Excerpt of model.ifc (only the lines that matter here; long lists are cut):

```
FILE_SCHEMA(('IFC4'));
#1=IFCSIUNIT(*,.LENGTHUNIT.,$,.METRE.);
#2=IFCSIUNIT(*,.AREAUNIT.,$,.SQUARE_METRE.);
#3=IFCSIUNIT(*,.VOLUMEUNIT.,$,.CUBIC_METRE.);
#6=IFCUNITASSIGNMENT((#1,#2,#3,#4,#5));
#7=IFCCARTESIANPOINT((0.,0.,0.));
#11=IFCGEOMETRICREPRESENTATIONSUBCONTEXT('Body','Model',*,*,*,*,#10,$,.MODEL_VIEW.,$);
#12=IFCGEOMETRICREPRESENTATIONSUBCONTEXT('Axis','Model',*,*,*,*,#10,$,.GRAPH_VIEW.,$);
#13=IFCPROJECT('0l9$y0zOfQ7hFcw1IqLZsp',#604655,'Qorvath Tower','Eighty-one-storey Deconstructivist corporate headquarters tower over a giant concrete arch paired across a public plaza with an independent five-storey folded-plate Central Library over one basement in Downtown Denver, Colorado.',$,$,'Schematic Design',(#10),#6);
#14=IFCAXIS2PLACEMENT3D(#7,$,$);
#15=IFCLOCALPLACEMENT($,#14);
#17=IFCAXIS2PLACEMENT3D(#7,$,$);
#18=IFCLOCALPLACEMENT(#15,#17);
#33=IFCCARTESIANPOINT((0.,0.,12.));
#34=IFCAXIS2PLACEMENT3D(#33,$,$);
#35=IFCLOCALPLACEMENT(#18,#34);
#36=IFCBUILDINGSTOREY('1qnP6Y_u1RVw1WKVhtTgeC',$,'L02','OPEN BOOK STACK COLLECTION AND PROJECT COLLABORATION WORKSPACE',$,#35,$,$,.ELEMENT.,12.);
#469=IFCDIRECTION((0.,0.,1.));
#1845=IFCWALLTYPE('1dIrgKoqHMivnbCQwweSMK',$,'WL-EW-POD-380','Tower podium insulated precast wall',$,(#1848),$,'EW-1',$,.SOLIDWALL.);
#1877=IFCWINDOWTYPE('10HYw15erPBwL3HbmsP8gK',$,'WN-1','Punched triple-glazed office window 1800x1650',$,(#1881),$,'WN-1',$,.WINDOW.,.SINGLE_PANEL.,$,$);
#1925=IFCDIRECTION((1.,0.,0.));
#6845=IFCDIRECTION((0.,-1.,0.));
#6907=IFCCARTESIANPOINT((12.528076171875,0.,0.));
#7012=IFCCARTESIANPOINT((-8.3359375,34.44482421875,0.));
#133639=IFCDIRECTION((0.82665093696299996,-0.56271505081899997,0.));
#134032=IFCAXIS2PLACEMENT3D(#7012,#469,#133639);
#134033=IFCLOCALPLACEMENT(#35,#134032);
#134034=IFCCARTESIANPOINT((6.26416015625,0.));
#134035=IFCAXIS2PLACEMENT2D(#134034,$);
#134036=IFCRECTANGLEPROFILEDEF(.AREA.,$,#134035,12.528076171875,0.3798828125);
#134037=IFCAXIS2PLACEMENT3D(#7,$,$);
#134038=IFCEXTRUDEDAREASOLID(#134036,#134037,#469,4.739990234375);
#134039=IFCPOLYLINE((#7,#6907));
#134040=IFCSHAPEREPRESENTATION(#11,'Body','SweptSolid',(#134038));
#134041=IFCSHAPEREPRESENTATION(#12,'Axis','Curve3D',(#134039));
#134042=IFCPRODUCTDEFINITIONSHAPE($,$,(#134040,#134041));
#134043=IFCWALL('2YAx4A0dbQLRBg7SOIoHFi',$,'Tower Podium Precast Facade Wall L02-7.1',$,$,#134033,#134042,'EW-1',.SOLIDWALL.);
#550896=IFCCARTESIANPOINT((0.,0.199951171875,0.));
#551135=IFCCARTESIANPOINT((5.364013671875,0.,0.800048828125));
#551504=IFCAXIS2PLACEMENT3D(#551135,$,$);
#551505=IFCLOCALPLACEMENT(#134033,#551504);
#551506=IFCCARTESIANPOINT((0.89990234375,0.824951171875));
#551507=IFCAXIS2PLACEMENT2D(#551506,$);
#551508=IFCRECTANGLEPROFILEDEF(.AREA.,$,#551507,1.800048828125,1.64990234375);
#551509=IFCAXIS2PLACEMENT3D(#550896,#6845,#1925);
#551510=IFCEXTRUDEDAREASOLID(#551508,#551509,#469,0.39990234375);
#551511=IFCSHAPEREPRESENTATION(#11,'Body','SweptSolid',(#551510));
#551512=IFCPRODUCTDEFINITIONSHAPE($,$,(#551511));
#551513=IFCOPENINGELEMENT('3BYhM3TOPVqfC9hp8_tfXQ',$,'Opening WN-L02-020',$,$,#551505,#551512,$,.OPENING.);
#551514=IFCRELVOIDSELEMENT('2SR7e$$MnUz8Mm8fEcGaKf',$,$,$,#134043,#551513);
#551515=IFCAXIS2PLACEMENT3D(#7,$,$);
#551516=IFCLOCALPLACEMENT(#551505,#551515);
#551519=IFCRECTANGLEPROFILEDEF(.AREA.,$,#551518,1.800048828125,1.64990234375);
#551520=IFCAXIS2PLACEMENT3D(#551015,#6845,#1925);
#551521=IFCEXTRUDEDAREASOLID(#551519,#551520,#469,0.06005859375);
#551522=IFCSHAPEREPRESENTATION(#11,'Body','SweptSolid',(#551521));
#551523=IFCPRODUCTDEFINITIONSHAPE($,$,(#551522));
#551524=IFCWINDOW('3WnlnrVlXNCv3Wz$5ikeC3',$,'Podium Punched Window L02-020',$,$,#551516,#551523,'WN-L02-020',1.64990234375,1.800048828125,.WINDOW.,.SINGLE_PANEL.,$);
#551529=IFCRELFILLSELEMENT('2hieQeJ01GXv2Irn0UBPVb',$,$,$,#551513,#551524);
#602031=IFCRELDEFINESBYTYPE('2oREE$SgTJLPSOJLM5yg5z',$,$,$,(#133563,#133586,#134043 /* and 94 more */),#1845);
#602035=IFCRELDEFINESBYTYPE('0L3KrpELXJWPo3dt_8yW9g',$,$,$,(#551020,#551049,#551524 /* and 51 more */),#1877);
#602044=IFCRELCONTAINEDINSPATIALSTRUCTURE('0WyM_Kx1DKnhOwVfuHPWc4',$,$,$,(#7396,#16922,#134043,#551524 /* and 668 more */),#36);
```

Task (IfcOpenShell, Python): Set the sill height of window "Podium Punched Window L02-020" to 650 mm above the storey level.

```python
import numpy as np
import ifcopenshell
import ifcopenshell.api.geometry
import ifcopenshell.geom
import ifcopenshell.util.element
import ifcopenshell.util.placement
import ifcopenshell.util.shape
import ifcopenshell.util.unit

model = ifcopenshell.open("model.ifc")
unit_scale = ifcopenshell.util.unit.calculate_unit_scale(model)

window = model.by_guid("3WnlnrVlXNCv3Wz$5ikeC3")
opening = window.FillsVoids[0].RelatingOpeningElement
storey = ifcopenshell.util.element.get_container(window, ifc_class="IfcBuildingStorey")
level = ifcopenshell.util.placement.get_local_placement(storey.ObjectPlacement)[2, 3]

# The opening's origin need not be at the sill, so measure its lowest point.
shape = ifcopenshell.geom.create_shape(ifcopenshell.geom.settings(), opening)
bottom = ifcopenshell.util.shape.get_shape_bottom_elevation(shape, shape.geometry) / unit_scale
dz = level + 0.65 - bottom

shift = np.array([0.0, 0.0, dz])
# The window is placed relative to its opening, so it follows when the opening moves.
matrix = ifcopenshell.util.placement.get_local_placement(opening.ObjectPlacement)
matrix[:3, 3] += shift
ifcopenshell.api.geometry.edit_object_placement(
    model, product=opening, matrix=matrix, is_si=False, should_transform_children=True
)

print(f"moved by {dz * unit_scale:+.3f} m")

model.write("model_updated.ifc")
```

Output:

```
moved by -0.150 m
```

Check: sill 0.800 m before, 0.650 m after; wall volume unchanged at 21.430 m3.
